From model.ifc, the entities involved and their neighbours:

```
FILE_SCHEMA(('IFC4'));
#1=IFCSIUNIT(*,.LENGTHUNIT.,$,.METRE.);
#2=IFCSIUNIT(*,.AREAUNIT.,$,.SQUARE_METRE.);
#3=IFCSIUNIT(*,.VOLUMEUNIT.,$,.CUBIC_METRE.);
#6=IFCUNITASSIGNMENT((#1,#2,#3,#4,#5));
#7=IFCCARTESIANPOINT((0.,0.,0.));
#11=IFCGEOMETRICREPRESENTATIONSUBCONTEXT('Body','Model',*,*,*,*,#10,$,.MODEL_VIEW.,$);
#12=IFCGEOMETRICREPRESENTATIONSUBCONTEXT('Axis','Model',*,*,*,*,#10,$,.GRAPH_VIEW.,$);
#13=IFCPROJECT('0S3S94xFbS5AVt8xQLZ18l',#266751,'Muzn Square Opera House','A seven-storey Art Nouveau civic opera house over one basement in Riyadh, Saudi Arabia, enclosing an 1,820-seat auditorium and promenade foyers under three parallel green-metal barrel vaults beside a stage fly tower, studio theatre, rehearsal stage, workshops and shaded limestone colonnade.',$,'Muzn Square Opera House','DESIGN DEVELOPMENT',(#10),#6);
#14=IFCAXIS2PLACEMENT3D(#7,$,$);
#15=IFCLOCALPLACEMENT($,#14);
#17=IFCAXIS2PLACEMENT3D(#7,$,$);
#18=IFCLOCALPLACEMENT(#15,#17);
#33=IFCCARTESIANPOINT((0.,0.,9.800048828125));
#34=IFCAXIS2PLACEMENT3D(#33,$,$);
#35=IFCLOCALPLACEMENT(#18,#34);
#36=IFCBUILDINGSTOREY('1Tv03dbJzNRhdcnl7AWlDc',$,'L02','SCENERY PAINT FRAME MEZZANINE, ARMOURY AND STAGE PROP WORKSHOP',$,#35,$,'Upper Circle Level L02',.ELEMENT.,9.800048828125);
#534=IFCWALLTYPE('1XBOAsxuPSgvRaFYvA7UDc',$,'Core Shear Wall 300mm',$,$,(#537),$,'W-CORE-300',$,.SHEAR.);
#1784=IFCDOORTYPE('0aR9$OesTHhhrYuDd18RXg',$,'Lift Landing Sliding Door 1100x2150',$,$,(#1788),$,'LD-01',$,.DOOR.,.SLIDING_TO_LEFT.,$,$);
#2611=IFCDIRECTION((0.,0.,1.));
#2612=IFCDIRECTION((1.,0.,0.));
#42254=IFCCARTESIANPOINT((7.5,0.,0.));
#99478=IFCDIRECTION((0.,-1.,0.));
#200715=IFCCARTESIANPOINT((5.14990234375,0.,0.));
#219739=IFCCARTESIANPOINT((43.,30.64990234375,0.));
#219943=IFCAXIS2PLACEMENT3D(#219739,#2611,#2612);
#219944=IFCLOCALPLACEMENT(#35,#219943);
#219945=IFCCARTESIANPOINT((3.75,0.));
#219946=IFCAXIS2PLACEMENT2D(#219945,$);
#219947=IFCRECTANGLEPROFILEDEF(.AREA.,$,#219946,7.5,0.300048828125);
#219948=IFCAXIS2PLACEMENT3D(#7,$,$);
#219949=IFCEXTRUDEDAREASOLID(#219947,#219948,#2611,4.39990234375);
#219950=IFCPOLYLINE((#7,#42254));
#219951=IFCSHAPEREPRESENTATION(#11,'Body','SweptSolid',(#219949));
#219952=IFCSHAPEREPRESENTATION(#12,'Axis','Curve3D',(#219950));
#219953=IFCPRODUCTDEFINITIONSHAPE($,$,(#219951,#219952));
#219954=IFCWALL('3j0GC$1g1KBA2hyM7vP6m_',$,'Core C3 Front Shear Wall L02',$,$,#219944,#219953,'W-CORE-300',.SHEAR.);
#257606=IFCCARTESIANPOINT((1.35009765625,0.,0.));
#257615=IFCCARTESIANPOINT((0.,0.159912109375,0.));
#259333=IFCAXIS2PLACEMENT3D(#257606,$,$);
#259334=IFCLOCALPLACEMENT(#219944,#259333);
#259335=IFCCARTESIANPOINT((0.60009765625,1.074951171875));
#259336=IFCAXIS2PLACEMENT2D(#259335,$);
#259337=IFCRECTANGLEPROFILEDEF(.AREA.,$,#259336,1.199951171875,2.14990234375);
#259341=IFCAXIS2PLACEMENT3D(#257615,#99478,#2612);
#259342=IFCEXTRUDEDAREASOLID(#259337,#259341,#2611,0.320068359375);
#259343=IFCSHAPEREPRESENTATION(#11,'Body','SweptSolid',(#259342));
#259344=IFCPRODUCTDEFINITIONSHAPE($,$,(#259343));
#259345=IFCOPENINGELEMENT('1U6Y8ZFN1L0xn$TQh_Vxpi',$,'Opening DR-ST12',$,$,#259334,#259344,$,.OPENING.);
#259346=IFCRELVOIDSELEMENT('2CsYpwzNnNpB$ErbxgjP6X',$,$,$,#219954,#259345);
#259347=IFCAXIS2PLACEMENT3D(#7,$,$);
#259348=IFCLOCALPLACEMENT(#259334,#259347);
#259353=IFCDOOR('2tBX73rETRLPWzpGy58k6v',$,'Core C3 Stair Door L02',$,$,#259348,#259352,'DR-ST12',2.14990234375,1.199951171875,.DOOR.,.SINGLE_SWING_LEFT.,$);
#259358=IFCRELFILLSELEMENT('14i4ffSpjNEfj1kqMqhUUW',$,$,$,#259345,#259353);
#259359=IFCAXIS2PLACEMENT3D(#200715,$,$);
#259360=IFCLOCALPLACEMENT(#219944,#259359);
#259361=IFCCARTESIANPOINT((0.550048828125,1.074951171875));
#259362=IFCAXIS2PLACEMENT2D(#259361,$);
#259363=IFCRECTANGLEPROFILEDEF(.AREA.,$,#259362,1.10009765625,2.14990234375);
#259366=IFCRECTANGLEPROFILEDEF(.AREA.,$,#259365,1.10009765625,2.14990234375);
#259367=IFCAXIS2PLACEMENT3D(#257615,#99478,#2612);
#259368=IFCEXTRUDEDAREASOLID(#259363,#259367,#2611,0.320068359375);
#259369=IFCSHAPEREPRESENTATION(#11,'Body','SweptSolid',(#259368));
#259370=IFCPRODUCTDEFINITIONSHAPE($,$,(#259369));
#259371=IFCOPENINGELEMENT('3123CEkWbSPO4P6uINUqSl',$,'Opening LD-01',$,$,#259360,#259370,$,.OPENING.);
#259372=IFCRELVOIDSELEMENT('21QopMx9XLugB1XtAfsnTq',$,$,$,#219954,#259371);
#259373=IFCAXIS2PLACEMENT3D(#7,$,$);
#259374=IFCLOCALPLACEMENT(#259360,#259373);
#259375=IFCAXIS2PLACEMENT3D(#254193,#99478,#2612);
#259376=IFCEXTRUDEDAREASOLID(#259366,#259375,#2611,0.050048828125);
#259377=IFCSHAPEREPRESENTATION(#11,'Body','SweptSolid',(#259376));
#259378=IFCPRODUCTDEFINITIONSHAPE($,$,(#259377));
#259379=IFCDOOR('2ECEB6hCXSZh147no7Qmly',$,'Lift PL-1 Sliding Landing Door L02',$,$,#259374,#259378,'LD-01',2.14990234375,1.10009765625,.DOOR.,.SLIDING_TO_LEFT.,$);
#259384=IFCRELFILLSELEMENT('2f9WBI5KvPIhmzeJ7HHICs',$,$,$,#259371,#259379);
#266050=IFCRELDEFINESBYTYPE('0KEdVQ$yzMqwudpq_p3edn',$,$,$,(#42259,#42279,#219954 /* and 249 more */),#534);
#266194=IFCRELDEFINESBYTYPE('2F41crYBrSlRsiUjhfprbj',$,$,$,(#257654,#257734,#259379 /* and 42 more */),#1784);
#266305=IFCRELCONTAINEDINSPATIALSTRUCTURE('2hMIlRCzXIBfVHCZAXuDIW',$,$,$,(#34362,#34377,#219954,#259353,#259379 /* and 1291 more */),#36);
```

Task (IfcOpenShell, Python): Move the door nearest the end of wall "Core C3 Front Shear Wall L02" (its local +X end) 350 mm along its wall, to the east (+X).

```python
import ifcopenshell
import ifcopenshell.api.geometry
import ifcopenshell.util.placement

model = ifcopenshell.open("model.ifc")

door = model.by_id(259379)
opening = door.FillsVoids[0].RelatingOpeningElement
wall = opening.VoidsElements[0].RelatingBuildingElement

wall_matrix = ifcopenshell.util.placement.get_local_placement(wall.ObjectPlacement)
shift = wall_matrix[:3, 0] * 0.35
before = ifcopenshell.util.placement.get_local_placement(door.ObjectPlacement)[:3, 3].copy()

# The door is placed relative to its opening, so it follows when the opening moves.
matrix = ifcopenshell.util.placement.get_local_placement(opening.ObjectPlacement)
matrix[:3, 3] += shift
ifcopenshell.api.geometry.edit_object_placement(
    model, product=opening, matrix=matrix, is_si=False, should_transform_children=True
)

after = ifcopenshell.util.placement.get_local_placement(door.ObjectPlacement)[:3, 3]
print("door moved by", (after - before).round(3) + 0.0)

model.write("model_v2.ifc")
```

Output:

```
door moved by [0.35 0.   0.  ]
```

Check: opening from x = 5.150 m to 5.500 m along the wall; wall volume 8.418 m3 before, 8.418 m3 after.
